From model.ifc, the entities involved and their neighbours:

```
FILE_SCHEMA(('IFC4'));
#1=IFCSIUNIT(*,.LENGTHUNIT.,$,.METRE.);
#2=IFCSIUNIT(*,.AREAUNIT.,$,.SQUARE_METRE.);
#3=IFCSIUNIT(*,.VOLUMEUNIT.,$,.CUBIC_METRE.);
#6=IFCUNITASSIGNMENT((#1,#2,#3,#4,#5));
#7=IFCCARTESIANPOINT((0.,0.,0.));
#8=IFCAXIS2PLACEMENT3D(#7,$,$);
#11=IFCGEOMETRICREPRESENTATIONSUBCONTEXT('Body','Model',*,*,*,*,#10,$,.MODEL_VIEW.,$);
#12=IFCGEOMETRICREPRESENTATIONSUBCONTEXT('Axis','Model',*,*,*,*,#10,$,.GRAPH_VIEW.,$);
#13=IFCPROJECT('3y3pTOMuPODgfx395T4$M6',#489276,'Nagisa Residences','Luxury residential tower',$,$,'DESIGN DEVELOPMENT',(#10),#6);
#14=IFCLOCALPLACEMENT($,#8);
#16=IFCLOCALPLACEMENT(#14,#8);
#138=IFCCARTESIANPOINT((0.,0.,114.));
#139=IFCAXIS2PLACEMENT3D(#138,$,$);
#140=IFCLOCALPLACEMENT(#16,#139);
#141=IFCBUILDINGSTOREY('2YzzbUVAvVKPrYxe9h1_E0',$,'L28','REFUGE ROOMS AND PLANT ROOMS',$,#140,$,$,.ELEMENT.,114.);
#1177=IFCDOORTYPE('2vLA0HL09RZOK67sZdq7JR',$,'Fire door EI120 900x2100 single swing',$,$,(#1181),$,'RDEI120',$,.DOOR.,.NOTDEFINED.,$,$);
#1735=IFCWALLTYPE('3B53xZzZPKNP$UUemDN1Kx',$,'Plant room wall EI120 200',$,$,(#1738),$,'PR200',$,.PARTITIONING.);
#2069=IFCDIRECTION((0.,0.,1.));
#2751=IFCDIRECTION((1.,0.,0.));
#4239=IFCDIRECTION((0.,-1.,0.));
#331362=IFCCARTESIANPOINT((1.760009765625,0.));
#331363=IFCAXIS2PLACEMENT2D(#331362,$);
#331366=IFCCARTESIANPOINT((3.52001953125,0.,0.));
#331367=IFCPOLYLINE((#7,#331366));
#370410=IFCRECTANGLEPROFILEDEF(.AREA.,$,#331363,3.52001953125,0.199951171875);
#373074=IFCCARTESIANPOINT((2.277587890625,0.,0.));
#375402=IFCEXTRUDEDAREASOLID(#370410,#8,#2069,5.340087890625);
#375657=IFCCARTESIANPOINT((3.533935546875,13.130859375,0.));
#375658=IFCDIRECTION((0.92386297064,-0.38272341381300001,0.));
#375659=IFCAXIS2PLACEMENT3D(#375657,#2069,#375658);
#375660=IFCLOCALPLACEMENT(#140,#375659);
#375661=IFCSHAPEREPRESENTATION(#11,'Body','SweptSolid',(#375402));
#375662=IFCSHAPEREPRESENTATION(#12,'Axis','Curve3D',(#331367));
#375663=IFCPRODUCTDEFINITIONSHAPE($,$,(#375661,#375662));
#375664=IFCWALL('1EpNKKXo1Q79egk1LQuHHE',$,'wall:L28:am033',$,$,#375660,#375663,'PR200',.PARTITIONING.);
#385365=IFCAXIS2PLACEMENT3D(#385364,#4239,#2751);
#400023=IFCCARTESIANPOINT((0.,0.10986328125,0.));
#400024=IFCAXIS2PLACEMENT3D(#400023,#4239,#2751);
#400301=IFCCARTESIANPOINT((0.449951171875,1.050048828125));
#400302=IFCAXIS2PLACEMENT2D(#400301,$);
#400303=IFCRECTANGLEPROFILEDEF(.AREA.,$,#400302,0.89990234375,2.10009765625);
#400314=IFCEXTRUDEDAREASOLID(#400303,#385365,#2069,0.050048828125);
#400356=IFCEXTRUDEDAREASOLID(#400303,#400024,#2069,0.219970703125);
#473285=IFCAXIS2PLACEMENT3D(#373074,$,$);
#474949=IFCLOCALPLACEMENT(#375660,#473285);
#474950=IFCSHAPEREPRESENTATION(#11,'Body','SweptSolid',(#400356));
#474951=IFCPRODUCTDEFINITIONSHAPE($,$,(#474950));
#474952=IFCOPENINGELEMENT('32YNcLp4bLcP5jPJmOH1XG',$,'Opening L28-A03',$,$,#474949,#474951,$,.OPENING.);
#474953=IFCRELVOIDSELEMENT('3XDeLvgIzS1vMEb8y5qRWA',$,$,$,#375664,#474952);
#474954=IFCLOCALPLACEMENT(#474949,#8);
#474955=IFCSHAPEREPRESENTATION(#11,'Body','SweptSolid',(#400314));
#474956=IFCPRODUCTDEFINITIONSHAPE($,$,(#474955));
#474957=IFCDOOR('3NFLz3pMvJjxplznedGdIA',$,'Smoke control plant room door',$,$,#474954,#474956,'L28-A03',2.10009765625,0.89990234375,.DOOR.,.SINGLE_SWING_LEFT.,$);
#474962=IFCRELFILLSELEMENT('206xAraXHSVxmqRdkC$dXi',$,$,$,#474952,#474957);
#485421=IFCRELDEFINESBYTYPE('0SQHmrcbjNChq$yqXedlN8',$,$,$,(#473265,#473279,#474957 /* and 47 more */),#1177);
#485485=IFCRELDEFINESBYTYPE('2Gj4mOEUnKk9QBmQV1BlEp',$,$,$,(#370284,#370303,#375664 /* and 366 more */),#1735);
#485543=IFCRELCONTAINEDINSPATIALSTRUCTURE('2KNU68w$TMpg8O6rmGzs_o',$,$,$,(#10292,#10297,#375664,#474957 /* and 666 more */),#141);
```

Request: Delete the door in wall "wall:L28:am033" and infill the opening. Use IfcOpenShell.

```python
import ifcopenshell
import ifcopenshell.api.feature
import ifcopenshell.api.root
import ifcopenshell.geom
import ifcopenshell.util.shape

model = ifcopenshell.open("model.ifc")
settings = ifcopenshell.geom.settings()


def volume(element):
    """Net volume in cubic metres, openings subtracted."""
    shape = ifcopenshell.geom.create_shape(settings, element)
    return ifcopenshell.util.shape.get_volume(shape.geometry)


door = model.by_guid("3NFLz3pMvJjxplznedGdIA")
opening = door.FillsVoids[0].RelatingOpeningElement
wall = opening.VoidsElements[0].RelatingBuildingElement
before = volume(wall)

ifcopenshell.api.root.remove_product(model, product=door)
ifcopenshell.api.feature.remove_feature(model, feature=opening)

after = volume(wall)

print(f"wall volume {before:.3f} -> {after:.3f} m3")

model.write("model-out.ifc")
```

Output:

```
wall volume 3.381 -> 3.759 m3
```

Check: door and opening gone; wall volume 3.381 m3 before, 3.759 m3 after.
